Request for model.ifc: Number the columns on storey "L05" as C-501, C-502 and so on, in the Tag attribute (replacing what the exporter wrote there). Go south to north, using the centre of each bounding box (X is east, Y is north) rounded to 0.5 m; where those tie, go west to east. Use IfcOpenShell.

First a look at what the model holds.

```python
import ifcopenshell
import ifcopenshell.util.element
import ifcopenshell.util.placement

model = ifcopenshell.open("model.ifc")
print(model.schema)
storey = next(s for s in model.by_type("IfcBuildingStorey") if s.Name == "L05")
columns = [e for e in ifcopenshell.util.element.get_decomposition(storey) if e.is_a("IfcColumn")]
for e in sorted(columns, key=lambda e: e.id()):
    origin = ifcopenshell.util.placement.get_local_placement(e.ObjectPlacement)[:3, 3]
    print(e.id(), e.Tag, e.Name, origin.round(2) + 0.0, sep=" | ")
```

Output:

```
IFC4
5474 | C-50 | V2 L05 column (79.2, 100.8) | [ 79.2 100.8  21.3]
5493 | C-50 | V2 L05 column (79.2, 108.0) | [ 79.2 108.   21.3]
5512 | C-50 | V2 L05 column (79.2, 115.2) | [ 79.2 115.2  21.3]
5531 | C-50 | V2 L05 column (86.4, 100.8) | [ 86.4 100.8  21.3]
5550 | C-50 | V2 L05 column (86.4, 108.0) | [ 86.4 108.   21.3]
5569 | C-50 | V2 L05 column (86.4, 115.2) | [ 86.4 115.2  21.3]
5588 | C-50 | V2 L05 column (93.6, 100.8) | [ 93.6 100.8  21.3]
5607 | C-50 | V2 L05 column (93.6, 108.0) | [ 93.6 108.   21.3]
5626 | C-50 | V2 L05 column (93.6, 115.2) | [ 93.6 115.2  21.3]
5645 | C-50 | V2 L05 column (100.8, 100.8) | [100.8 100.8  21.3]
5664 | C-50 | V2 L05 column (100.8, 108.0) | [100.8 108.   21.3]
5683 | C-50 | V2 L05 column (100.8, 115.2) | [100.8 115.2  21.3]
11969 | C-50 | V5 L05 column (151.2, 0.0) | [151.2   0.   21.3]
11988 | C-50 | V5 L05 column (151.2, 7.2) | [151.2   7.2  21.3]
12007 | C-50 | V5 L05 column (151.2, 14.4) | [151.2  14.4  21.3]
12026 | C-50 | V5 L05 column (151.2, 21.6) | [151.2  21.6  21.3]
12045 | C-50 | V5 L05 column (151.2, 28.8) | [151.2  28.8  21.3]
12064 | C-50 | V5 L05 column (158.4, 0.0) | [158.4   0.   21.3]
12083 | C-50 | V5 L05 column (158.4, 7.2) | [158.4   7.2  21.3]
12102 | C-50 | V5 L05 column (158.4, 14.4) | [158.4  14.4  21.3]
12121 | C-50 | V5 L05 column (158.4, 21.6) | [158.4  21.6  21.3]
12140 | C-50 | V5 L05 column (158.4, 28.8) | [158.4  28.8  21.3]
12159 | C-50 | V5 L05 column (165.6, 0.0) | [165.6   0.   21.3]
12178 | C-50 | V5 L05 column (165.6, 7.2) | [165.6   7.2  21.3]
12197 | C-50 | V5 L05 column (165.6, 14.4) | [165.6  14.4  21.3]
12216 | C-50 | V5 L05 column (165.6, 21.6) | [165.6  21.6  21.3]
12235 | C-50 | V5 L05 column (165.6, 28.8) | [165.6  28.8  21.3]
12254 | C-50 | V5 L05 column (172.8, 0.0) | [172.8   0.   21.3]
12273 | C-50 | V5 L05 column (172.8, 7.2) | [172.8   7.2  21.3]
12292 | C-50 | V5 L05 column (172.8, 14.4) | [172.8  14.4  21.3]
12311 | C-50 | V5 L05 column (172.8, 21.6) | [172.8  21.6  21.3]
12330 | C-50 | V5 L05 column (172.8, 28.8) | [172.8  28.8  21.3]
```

```python
import ifcopenshell
import ifcopenshell.geom
import ifcopenshell.util.element
import ifcopenshell.util.shape

model = ifcopenshell.open("model.ifc")
settings = ifcopenshell.geom.settings()
settings.set("use-world-coords", True)


def centre(element):
    shape = ifcopenshell.geom.create_shape(settings, element)
    return ifcopenshell.util.shape.get_bbox_centroid(shape.geometry)


storey = next(s for s in model.by_type("IfcBuildingStorey") if s.Name == "L05")
columns = [e for e in ifcopenshell.util.element.get_decomposition(storey) if e.is_a("IfcColumn")]

# Insertion points can sit at a corner or the storey origin, so sort by the geometry (in metres).
centres = {e: centre(e) for e in columns}
columns.sort(key=lambda e: (round(centres[e][1] / 0.5), centres[e][0]))

for i, e in enumerate(columns, start=1):
    number = f"C-5{i:02d}"
    e.Tag = number
    print(e.id(), number)

model.write("model_updated.ifc")
```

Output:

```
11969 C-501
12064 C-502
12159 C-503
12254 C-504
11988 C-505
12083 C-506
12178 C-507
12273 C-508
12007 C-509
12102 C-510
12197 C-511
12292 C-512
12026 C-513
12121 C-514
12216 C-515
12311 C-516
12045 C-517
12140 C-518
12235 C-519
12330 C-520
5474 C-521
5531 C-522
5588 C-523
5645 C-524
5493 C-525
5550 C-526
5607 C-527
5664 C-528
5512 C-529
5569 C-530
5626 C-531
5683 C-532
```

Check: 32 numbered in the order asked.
